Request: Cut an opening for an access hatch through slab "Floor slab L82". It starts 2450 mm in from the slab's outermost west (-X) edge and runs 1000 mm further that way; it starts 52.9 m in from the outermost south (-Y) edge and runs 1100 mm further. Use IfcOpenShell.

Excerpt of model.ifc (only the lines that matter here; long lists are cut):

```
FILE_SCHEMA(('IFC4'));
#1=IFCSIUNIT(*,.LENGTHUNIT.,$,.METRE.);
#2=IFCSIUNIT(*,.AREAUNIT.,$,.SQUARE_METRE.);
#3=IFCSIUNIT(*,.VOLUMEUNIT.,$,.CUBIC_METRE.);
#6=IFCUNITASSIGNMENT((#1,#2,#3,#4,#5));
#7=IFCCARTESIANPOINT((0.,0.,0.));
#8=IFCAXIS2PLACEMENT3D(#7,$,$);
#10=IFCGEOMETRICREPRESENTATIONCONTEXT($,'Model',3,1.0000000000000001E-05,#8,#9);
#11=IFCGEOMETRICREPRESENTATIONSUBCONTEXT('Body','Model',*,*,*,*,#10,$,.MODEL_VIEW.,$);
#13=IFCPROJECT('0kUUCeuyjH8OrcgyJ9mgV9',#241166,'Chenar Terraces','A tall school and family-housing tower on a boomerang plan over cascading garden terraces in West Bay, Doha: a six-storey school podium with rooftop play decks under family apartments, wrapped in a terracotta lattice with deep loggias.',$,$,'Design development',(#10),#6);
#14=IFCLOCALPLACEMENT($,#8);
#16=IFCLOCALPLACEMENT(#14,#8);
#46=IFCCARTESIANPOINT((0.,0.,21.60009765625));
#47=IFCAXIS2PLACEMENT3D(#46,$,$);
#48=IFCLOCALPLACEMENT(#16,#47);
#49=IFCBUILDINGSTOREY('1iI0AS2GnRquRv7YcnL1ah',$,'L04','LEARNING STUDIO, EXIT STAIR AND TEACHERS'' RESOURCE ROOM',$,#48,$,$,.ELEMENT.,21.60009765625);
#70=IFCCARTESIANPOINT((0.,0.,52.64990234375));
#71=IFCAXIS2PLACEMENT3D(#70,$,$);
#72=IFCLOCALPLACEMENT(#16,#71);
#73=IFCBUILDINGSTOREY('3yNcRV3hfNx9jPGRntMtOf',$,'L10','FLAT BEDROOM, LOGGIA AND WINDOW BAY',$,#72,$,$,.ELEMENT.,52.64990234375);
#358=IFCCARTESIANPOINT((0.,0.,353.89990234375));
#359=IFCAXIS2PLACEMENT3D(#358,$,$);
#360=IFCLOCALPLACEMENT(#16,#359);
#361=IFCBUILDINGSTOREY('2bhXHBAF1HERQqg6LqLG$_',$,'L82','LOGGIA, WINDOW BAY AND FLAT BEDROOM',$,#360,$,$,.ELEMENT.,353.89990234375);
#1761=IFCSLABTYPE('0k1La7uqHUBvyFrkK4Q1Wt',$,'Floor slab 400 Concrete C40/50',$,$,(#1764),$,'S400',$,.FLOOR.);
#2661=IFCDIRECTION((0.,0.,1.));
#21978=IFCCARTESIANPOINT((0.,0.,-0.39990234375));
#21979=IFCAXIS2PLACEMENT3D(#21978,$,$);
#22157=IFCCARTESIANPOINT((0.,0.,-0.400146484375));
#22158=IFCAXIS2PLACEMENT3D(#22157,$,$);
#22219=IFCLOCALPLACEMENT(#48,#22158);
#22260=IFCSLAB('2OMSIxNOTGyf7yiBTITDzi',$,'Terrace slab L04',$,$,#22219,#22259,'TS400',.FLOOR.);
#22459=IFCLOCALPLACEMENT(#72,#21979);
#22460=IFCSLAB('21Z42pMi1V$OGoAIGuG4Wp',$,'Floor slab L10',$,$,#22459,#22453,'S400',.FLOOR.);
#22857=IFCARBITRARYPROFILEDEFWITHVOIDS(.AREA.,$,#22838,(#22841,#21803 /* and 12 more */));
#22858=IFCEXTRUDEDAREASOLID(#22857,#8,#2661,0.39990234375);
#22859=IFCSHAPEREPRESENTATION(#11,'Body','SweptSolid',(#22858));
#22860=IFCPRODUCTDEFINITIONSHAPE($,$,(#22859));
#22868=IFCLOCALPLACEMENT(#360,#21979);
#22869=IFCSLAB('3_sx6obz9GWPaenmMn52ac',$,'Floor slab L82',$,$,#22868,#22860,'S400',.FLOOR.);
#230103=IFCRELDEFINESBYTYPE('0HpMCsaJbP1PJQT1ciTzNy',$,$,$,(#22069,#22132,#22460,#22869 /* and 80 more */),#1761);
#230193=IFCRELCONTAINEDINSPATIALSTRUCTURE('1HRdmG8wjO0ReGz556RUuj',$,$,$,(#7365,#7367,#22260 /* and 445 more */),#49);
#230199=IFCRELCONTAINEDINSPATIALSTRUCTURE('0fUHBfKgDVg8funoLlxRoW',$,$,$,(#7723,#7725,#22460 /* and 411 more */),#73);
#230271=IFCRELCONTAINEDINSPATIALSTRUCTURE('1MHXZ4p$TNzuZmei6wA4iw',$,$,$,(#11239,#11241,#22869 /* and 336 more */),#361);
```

```python
import numpy as np
import ifcopenshell
import ifcopenshell.api.feature
import ifcopenshell.api.geometry
import ifcopenshell.api.root
import ifcopenshell.geom
import ifcopenshell.util.placement
import ifcopenshell.util.representation
import ifcopenshell.util.shape
import ifcopenshell.util.unit

model = ifcopenshell.open("model.ifc")
unit_scale = ifcopenshell.util.unit.calculate_unit_scale(model)
settings = ifcopenshell.geom.settings()


def volume(element):
    """Net volume in cubic metres, openings subtracted."""
    shape = ifcopenshell.geom.create_shape(settings, element)
    return ifcopenshell.util.shape.get_volume(shape.geometry)


slab = model.by_guid("3_sx6obz9GWPaenmMn52ac")
before = volume(slab)

# Extent in the slab's own axes, in metres. The edges named are its -X and -Y sides.
slab_shape = ifcopenshell.geom.create_shape(settings, slab)
vertices = ifcopenshell.util.shape.get_vertices(slab_shape.geometry)
x_min, y_min, bottom = vertices.min(axis=0)
top = vertices[:, 2].max()

opening = ifcopenshell.api.root.create_entity(model, ifc_class="IfcOpeningElement", name="Access hatch opening", predefined_type="OPENING")
context = ifcopenshell.util.representation.get_context(model, "Model", "Body", "MODEL_VIEW")
width, depth = 1, 1.1
outline = [(0.0, 0.0), (width, 0.0), (width, depth), (0.0, depth), (0.0, 0.0)]
# Overshoot both faces by 50 mm so the cut is clean.
shape = ifcopenshell.api.geometry.add_slab_representation(
    model, context=context, depth=top - bottom + 0.1, polyline=outline
)
ifcopenshell.api.geometry.assign_representation(model, product=opening, representation=shape)

matrix = ifcopenshell.util.placement.get_local_placement(slab.ObjectPlacement)
matrix[:, 3] = matrix @ np.append(np.array([x_min + 2.45, y_min + 52.9, bottom - 0.05]) / unit_scale, 1.0)
ifcopenshell.api.geometry.edit_object_placement(model, product=opening, matrix=matrix, is_si=False)
ifcopenshell.api.feature.add_feature(model, feature=opening, element=slab)

after = volume(slab)

print(f"slab volume {before:.3f} -> {after:.3f} m3")

model.write("model_edited.ifc")
```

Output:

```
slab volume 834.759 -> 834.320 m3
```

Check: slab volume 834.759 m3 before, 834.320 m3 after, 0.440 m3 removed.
